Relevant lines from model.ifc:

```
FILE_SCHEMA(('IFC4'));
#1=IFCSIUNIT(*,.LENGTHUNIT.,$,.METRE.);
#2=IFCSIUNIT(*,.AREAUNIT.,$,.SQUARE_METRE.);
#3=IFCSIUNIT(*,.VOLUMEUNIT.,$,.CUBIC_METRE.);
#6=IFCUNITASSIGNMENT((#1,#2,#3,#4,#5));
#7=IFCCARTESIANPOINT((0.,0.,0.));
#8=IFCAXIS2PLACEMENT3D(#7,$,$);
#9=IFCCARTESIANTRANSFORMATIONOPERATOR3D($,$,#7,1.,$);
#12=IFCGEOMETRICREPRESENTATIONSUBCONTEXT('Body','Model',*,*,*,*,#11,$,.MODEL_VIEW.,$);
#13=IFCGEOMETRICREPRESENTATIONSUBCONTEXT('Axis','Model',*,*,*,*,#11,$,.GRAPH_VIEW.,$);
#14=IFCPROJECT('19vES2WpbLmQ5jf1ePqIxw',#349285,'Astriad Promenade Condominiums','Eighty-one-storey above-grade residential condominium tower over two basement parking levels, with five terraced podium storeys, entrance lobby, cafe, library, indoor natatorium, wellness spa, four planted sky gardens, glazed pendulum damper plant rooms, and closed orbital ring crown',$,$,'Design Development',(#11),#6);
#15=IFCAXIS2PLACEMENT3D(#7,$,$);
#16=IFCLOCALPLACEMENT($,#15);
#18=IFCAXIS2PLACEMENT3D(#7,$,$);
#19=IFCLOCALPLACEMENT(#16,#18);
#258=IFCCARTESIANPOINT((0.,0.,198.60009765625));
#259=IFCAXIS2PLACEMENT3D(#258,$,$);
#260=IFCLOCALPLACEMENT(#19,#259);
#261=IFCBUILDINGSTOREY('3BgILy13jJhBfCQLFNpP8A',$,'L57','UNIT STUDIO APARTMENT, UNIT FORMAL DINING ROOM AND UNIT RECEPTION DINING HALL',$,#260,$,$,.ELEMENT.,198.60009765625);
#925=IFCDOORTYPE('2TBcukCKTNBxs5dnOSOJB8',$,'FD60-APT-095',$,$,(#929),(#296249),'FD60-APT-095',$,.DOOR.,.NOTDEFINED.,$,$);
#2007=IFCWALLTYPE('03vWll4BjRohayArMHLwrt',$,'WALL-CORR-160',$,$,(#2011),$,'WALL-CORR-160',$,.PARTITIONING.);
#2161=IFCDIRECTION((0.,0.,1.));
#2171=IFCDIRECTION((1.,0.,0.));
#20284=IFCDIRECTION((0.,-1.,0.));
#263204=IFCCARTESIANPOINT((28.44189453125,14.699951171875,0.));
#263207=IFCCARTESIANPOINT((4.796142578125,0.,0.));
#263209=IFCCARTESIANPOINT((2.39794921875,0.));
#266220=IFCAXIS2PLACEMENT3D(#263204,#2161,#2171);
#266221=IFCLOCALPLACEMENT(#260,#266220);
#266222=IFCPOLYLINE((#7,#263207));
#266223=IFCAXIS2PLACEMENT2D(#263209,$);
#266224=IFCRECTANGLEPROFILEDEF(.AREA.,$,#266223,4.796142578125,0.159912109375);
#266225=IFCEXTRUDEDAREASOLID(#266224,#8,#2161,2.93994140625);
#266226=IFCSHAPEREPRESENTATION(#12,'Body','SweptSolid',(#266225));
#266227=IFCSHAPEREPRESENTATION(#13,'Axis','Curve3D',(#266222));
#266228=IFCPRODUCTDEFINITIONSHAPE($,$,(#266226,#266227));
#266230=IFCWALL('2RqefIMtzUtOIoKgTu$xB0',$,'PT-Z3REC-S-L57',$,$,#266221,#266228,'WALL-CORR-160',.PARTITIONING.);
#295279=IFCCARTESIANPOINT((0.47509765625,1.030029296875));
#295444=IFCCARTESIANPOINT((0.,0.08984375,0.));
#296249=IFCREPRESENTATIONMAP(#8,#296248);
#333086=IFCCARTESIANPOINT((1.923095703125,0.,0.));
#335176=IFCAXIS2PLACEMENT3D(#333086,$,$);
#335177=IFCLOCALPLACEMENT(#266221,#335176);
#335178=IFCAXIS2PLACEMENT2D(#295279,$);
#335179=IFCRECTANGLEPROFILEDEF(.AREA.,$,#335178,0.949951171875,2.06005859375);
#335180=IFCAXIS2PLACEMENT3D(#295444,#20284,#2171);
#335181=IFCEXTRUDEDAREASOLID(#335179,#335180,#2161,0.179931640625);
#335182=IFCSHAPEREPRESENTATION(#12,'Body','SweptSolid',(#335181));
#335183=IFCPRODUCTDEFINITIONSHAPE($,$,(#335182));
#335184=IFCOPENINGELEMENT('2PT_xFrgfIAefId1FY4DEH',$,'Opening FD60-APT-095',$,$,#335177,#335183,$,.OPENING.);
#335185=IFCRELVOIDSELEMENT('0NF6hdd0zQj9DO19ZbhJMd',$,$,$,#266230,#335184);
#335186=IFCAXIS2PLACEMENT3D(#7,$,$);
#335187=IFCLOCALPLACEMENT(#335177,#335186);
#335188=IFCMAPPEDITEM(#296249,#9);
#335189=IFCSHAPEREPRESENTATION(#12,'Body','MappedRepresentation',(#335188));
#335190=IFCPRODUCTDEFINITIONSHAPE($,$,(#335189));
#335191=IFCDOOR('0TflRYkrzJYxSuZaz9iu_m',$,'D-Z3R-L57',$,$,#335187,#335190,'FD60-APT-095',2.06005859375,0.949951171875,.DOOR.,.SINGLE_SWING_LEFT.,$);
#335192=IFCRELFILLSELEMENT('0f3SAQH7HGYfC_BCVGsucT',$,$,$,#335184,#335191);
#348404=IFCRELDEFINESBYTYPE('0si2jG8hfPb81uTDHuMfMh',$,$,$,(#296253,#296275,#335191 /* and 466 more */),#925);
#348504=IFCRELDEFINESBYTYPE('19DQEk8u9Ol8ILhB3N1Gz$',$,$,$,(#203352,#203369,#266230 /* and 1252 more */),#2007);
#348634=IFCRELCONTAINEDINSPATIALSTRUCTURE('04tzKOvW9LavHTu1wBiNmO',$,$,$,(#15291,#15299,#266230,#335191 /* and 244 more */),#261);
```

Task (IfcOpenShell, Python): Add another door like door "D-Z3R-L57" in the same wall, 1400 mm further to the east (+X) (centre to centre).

```python
import ifcopenshell
import ifcopenshell.api.feature
import ifcopenshell.api.geometry
import ifcopenshell.api.root
import ifcopenshell.geom
import ifcopenshell.util.element
import ifcopenshell.util.placement
import ifcopenshell.util.shape
import ifcopenshell.util.unit

model = ifcopenshell.open("model.ifc")
unit_scale = ifcopenshell.util.unit.calculate_unit_scale(model)
settings = ifcopenshell.geom.settings()


def volume(element):
    """Net volume in cubic metres, openings subtracted."""
    shape = ifcopenshell.geom.create_shape(settings, element)
    return ifcopenshell.util.shape.get_volume(shape.geometry)


door = model.by_id(335191)
opening = door.FillsVoids[0].RelatingOpeningElement
wall = opening.VoidsElements[0].RelatingBuildingElement
before = volume(wall)
shift = ifcopenshell.util.placement.get_local_placement(wall.ObjectPlacement)[:3, 0] * 1.4 / unit_scale

# copy_class copies the void relationship, type, container and properties, but no geometry.
new_opening = ifcopenshell.api.root.copy_class(model, product=opening)
new_opening.Representation = ifcopenshell.util.element.copy_deep(
    model, opening.Representation, exclude=["IfcGeometricRepresentationContext", "IfcRepresentationMap"]
)
new_door = ifcopenshell.api.root.copy_class(model, product=door)
new_door.Representation = ifcopenshell.util.element.copy_deep(
    model, door.Representation, exclude=["IfcGeometricRepresentationContext", "IfcRepresentationMap"]
)
new_door.Tag = None
ifcopenshell.api.feature.add_filling(model, opening=new_opening, element=new_door)

for old, new in ((opening, new_opening), (door, new_door)):
    matrix = ifcopenshell.util.placement.get_local_placement(old.ObjectPlacement)
    matrix[:3, 3] += shift
    ifcopenshell.api.geometry.edit_object_placement(model, product=new, matrix=matrix, is_si=False)

after = volume(wall)

print(f"wall volume {before:.3f} -> {after:.3f} m3")

model.write("model_v2.ifc")
```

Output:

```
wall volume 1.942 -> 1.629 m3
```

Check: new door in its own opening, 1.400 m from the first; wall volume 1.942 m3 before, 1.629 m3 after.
